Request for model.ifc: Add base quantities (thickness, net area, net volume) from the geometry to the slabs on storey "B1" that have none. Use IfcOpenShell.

First a look at what the model holds.

```python
import ifcopenshell
import ifcopenshell.util.element
import ifcopenshell.util.unit

model = ifcopenshell.open("model.ifc")
print(model.schema)
for unit_type in ("LENGTHUNIT", "AREAUNIT", "VOLUMEUNIT"):
    print(unit_type, ifcopenshell.util.unit.calculate_unit_scale(model, unit_type))
storey = next(s for s in model.by_type("IfcBuildingStorey") if s.Name == "B1")
slabs = [e for e in ifcopenshell.util.element.get_decomposition(storey) if e.is_a("IfcSlab")]
for e in sorted(slabs, key=lambda e: e.id()):
    print(e.id(), e.is_a(), e.Name, list(ifcopenshell.util.element.get_psets(e, qtos_only=True)), sep=" | ")
```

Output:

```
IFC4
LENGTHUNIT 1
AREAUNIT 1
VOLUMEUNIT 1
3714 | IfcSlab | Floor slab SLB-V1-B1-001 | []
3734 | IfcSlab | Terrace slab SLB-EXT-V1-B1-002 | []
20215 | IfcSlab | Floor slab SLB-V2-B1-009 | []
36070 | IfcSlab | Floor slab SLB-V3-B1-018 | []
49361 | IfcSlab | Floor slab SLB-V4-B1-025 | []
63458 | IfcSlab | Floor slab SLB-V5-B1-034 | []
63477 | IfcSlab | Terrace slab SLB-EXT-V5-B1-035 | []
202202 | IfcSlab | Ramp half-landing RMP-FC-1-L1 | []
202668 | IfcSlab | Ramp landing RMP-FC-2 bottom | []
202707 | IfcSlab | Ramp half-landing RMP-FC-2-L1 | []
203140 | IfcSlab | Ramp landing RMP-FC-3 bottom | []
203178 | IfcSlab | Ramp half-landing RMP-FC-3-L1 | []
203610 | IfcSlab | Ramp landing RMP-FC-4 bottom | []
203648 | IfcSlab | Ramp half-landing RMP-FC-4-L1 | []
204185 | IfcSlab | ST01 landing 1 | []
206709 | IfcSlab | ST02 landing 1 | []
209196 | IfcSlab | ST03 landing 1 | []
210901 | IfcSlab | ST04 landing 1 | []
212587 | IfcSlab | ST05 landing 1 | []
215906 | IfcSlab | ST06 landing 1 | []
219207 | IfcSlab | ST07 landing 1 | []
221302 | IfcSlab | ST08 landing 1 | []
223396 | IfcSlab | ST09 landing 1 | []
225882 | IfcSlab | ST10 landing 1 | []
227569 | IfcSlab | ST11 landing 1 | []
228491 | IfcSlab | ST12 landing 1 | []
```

```python
import ifcopenshell
import ifcopenshell.api.pset
import ifcopenshell.geom
import ifcopenshell.util.element
import ifcopenshell.util.shape
import ifcopenshell.util.unit

model = ifcopenshell.open("model.ifc")
unit_scale = ifcopenshell.util.unit.calculate_unit_scale(model)
area_scale = ifcopenshell.util.unit.calculate_unit_scale(model, "AREAUNIT")
volume_scale = ifcopenshell.util.unit.calculate_unit_scale(model, "VOLUMEUNIT")
settings = ifcopenshell.geom.settings()

storey = next(s for s in model.by_type("IfcBuildingStorey") if s.Name == "B1")
slabs = [e for e in ifcopenshell.util.element.get_decomposition(storey) if e.is_a("IfcSlab")]

for e in sorted(slabs, key=lambda e: e.id()):
    if ifcopenshell.util.element.get_psets(e, qtos_only=True, should_inherit=False):
        continue
    # Geometry comes back in metres, in the element's own axes.
    shape = ifcopenshell.geom.create_shape(settings, e)
    values = {
        "Width": ifcopenshell.util.shape.get_z(shape.geometry) / unit_scale,
        "NetArea": ifcopenshell.util.shape.get_footprint_area(shape.geometry) / area_scale,
        "NetVolume": ifcopenshell.util.shape.get_volume(shape.geometry) / volume_scale,
    }
    qto = ifcopenshell.api.pset.add_qto(model, product=e, name="Qto_SlabBaseQuantities")
    ifcopenshell.api.pset.edit_qto(model, qto=qto, properties=values)
    print(e.id(), {k: round(v, 3) for k, v in values.items()})

model.write("model-out.ifc")
```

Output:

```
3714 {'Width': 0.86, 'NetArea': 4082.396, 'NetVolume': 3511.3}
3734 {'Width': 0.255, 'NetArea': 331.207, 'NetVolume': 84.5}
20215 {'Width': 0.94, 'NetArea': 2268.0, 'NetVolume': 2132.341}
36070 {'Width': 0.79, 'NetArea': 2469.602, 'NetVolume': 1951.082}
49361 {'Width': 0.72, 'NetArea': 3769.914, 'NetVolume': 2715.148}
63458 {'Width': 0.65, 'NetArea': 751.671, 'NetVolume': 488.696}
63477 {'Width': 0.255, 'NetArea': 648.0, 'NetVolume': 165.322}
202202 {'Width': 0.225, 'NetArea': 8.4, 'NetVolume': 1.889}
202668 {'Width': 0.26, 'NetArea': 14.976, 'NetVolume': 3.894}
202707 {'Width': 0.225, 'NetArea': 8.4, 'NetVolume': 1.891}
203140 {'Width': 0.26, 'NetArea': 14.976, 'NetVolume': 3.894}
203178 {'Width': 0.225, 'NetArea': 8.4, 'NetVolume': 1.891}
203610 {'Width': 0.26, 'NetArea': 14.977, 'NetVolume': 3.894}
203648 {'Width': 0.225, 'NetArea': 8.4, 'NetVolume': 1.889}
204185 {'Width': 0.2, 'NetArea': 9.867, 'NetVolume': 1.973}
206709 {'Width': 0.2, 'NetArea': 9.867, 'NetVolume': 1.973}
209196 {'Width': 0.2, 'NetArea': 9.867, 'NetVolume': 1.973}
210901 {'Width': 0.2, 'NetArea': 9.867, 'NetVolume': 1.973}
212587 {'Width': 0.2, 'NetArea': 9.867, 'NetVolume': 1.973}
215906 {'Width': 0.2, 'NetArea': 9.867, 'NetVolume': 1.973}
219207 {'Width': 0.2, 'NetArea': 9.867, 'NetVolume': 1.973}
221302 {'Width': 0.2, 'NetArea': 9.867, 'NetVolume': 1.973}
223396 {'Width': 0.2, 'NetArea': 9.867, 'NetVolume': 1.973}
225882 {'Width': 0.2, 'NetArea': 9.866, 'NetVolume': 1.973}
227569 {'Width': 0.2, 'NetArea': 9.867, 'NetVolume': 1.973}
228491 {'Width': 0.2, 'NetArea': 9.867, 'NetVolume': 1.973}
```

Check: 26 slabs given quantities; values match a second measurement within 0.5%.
